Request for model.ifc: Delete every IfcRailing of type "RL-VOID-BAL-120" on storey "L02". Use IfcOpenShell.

First a look at what the model holds.

```python
import ifcopenshell
import ifcopenshell.util.element

model = ifcopenshell.open("model.ifc")
print(model.schema)
storey = next(s for s in model.by_type("IfcBuildingStorey") if s.Name == "L02")
railings = [e for e in ifcopenshell.util.element.get_decomposition(storey) if e.is_a("IfcRailing")]
seen = {}
for e in railings:
    element_type = ifcopenshell.util.element.get_type(e)
    name = element_type.Name if element_type not in (None, e) else None
    seen[name] = seen.get(name, 0) + 1
for name, count in sorted(seen.items(), key=str):
    print(count, "x", name)
```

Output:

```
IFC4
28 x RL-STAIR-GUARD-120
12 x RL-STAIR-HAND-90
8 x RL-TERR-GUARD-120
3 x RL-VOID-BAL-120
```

```python
import ifcopenshell
import ifcopenshell.api.root
import ifcopenshell.util.element

model = ifcopenshell.open("model.ifc")

storey = next(s for s in model.by_type("IfcBuildingStorey") if s.Name == "L02")
railings = [e for e in ifcopenshell.util.element.get_decomposition(storey) if e.is_a("IfcRailing")]
targets = [e for e in railings if (t := ifcopenshell.util.element.get_type(e)) not in (None, e) and t.Name == "RL-VOID-BAL-120"]

for e in targets:
    ifcopenshell.api.root.remove_product(model, product=e)
print(len(targets), "removed")

model.write("model-out.ifc")
```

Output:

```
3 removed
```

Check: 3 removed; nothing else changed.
